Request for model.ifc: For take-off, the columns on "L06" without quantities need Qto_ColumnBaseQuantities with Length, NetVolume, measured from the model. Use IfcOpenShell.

First a look at what the model holds.

```python
import ifcopenshell
import ifcopenshell.util.element
import ifcopenshell.util.unit

model = ifcopenshell.open("model.ifc")
print(model.schema)
for unit_type in ("LENGTHUNIT", "AREAUNIT", "VOLUMEUNIT"):
    print(unit_type, ifcopenshell.util.unit.calculate_unit_scale(model, unit_type))
storey = next(s for s in model.by_type("IfcBuildingStorey") if s.Name == "L06")
columns = [e for e in ifcopenshell.util.element.get_decomposition(storey) if e.is_a("IfcColumn")]
for e in sorted(columns, key=lambda e: e.id()):
    print(e.id(), e.is_a(), e.Name, list(ifcopenshell.util.element.get_psets(e, qtos_only=True)), sep=" | ")
```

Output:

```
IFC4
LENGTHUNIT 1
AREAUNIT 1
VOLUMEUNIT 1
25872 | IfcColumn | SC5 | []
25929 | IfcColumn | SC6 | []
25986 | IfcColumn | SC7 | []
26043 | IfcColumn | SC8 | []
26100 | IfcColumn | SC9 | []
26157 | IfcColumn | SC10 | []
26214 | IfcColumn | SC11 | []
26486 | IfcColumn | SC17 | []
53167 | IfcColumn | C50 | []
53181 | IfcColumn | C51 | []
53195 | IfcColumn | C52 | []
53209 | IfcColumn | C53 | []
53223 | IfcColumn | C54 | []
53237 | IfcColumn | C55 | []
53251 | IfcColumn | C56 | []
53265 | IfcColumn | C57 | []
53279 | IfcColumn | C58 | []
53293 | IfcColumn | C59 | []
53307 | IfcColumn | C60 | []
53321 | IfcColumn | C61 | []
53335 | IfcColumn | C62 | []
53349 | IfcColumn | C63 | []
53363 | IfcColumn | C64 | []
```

```python
import ifcopenshell
import ifcopenshell.api.pset
import ifcopenshell.geom
import ifcopenshell.util.element
import ifcopenshell.util.shape
import ifcopenshell.util.unit

model = ifcopenshell.open("model.ifc")
unit_scale = ifcopenshell.util.unit.calculate_unit_scale(model)
volume_scale = ifcopenshell.util.unit.calculate_unit_scale(model, "VOLUMEUNIT")
settings = ifcopenshell.geom.settings()

storey = next(s for s in model.by_type("IfcBuildingStorey") if s.Name == "L06")
columns = [e for e in ifcopenshell.util.element.get_decomposition(storey) if e.is_a("IfcColumn")]

for e in sorted(columns, key=lambda e: e.id()):
    if ifcopenshell.util.element.get_psets(e, qtos_only=True, should_inherit=False):
        continue
    # Geometry comes back in metres, in the element's own axes.
    shape = ifcopenshell.geom.create_shape(settings, e)
    values = {
        "Length": ifcopenshell.util.shape.get_z(shape.geometry) / unit_scale,
        "NetVolume": ifcopenshell.util.shape.get_volume(shape.geometry) / volume_scale,
    }
    qto = ifcopenshell.api.pset.add_qto(model, product=e, name="Qto_ColumnBaseQuantities")
    ifcopenshell.api.pset.edit_qto(model, qto=qto, properties=values)
    print(e.id(), {k: round(v, 3) for k, v in values.items()})

model.write("model_edited.ifc")
```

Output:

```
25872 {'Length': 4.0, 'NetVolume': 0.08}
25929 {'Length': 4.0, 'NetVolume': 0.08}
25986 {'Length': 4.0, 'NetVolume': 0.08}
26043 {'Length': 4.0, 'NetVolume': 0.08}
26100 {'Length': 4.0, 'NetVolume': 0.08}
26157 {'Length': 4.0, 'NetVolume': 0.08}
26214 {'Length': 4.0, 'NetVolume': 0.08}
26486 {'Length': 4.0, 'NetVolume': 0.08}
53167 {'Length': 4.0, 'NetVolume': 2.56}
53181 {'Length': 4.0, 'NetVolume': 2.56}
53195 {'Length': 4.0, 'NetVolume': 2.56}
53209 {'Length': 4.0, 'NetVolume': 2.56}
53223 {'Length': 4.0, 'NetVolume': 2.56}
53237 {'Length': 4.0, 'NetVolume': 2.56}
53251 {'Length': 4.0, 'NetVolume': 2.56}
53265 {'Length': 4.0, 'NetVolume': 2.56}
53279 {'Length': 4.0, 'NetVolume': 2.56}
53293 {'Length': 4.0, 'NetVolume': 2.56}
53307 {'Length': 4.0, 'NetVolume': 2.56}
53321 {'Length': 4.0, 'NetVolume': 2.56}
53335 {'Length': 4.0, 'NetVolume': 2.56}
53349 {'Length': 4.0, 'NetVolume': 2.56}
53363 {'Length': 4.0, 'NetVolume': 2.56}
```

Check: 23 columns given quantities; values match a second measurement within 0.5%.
